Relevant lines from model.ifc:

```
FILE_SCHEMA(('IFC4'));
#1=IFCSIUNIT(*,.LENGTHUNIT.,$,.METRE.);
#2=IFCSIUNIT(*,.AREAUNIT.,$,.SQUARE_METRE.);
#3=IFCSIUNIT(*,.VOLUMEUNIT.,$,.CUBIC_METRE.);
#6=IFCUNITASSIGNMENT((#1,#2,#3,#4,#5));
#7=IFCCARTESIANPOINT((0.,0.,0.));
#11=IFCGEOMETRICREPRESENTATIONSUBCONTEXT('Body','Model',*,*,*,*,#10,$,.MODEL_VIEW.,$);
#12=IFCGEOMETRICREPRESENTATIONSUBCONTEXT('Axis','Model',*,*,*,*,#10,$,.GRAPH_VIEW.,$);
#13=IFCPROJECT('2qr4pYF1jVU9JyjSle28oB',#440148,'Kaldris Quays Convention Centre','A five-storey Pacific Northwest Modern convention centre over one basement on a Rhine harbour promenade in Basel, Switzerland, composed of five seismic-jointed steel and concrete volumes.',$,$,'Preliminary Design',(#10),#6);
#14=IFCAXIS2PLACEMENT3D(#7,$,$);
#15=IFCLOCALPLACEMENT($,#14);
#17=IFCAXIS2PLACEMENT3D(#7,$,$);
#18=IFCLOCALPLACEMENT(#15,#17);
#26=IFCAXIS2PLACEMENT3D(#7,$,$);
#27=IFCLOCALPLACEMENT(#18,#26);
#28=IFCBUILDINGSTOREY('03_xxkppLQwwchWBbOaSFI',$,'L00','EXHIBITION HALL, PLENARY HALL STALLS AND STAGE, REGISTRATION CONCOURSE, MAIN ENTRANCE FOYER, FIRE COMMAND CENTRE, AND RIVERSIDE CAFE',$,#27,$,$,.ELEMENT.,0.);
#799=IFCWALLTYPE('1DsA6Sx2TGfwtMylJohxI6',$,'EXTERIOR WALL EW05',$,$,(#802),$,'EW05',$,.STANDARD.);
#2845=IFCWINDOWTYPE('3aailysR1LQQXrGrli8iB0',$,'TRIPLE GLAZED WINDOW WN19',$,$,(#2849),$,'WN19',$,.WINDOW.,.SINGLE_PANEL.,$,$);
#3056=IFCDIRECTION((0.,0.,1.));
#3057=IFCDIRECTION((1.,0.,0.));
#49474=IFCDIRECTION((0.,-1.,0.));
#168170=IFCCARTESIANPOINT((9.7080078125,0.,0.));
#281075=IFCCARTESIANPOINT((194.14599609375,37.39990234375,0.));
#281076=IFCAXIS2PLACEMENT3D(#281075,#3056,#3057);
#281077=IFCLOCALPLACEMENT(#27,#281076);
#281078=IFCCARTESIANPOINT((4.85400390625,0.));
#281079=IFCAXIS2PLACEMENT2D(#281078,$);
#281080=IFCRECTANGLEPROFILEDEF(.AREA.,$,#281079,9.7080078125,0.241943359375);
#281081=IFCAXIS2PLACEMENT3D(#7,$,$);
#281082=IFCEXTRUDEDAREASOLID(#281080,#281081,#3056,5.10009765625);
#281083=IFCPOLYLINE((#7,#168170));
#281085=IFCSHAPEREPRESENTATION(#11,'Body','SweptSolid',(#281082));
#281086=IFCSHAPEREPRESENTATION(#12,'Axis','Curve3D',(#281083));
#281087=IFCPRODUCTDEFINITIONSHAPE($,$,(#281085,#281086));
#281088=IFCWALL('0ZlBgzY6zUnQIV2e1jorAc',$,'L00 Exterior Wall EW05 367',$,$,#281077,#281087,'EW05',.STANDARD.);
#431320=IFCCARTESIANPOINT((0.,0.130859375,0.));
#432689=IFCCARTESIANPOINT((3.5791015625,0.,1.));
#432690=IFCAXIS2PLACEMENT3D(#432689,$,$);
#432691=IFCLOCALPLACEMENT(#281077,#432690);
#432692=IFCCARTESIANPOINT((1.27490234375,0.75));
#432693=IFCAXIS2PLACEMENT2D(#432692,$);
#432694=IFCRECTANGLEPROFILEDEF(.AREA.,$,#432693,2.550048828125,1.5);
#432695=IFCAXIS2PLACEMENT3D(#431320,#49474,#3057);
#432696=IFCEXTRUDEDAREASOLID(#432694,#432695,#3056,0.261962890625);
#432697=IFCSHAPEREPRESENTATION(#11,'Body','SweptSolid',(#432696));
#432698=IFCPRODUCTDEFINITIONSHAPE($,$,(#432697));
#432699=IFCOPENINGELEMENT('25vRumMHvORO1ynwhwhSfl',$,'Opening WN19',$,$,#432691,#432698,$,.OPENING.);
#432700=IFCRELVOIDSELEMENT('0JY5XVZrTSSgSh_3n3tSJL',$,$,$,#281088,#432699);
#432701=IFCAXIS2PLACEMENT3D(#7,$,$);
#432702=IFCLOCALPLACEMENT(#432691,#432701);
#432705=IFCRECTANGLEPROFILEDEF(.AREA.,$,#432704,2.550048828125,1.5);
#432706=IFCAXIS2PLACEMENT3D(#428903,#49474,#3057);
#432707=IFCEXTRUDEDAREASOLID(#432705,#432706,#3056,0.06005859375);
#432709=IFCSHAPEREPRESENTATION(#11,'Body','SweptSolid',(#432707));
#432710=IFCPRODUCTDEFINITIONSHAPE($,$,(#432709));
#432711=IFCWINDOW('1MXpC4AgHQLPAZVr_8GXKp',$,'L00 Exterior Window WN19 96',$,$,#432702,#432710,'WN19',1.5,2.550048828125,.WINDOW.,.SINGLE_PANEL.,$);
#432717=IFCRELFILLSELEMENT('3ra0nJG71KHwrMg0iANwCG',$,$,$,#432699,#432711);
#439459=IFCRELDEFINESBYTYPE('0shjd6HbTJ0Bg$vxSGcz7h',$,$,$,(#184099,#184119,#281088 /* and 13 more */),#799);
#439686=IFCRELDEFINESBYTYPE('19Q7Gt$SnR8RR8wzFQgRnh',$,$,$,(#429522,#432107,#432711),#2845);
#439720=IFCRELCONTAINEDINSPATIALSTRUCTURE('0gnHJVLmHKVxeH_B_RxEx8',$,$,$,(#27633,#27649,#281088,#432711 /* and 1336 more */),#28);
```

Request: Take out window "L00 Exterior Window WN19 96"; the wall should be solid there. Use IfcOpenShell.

```python
import ifcopenshell
import ifcopenshell.api.feature
import ifcopenshell.api.root
import ifcopenshell.geom
import ifcopenshell.util.shape

model = ifcopenshell.open("model.ifc")
settings = ifcopenshell.geom.settings()


def volume(element):
    """Net volume in cubic metres, openings subtracted."""
    shape = ifcopenshell.geom.create_shape(settings, element)
    return ifcopenshell.util.shape.get_volume(shape.geometry)


window = model.by_guid("1MXpC4AgHQLPAZVr_8GXKp")
opening = window.FillsVoids[0].RelatingOpeningElement
wall = opening.VoidsElements[0].RelatingBuildingElement
before = volume(wall)

ifcopenshell.api.root.remove_product(model, product=window)
ifcopenshell.api.feature.remove_feature(model, feature=opening)

after = volume(wall)

print(f"wall volume {before:.3f} -> {after:.3f} m3")

model.write("model_rev.ifc")
```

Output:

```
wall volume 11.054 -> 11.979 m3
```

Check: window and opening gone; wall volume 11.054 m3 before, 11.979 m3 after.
